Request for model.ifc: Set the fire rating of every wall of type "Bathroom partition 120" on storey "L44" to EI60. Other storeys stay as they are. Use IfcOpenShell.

First a look at what the model holds.

```python
import ifcopenshell
import ifcopenshell.util.element

model = ifcopenshell.open("model.ifc")
print(model.schema)
storey = next(s for s in model.by_type("IfcBuildingStorey") if s.Name == "L44")
walls = [e for e in ifcopenshell.util.element.get_decomposition(storey) if e.is_a("IfcWall")]
seen = {}
for e in walls:
    element_type = ifcopenshell.util.element.get_type(e)
    key = (element_type.Name if element_type != e and element_type else None, ifcopenshell.util.element.get_pset(e, "Pset_WallCommon", "FireRating"))
    seen[key] = seen.get(key, 0) + 1
for (name, value), count in sorted(seen.items(), key=str):
    print(count, "x", name, "|", value)
```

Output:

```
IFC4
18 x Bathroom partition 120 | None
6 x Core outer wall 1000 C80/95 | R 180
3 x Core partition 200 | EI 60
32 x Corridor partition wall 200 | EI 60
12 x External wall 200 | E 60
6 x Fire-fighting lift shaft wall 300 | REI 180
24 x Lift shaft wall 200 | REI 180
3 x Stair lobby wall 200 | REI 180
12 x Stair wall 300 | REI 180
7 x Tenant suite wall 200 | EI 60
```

```python
import ifcopenshell
import ifcopenshell.api.pset
import ifcopenshell.util.element

model = ifcopenshell.open("model.ifc")

storey = next(s for s in model.by_type("IfcBuildingStorey") if s.Name == "L44")
walls = [e for e in ifcopenshell.util.element.get_decomposition(storey) if e.is_a("IfcWall")]

count = 0
for e in walls:
    element_type = ifcopenshell.util.element.get_type(e)
    if element_type in (None, e) or element_type.Name != "Bathroom partition 120":
        continue
    found = ifcopenshell.util.element.get_pset(e, "Pset_WallCommon", should_inherit=False)
    if found:
        pset = model.by_id(found["id"])
        if len(ifcopenshell.util.element.get_elements_by_pset(pset)) > 1:
            pset = ifcopenshell.api.pset.unshare_pset(model, products=[e], pset=pset)[0]
    else:
        pset = ifcopenshell.api.pset.add_pset(model, product=e, name="Pset_WallCommon")
    ifcopenshell.api.pset.edit_pset(model, pset=pset, properties={"FireRating": "EI60"})
    count += 1

print(count, "walls updated")

model.write("model-out.ifc")
```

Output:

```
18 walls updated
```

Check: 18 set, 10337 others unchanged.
